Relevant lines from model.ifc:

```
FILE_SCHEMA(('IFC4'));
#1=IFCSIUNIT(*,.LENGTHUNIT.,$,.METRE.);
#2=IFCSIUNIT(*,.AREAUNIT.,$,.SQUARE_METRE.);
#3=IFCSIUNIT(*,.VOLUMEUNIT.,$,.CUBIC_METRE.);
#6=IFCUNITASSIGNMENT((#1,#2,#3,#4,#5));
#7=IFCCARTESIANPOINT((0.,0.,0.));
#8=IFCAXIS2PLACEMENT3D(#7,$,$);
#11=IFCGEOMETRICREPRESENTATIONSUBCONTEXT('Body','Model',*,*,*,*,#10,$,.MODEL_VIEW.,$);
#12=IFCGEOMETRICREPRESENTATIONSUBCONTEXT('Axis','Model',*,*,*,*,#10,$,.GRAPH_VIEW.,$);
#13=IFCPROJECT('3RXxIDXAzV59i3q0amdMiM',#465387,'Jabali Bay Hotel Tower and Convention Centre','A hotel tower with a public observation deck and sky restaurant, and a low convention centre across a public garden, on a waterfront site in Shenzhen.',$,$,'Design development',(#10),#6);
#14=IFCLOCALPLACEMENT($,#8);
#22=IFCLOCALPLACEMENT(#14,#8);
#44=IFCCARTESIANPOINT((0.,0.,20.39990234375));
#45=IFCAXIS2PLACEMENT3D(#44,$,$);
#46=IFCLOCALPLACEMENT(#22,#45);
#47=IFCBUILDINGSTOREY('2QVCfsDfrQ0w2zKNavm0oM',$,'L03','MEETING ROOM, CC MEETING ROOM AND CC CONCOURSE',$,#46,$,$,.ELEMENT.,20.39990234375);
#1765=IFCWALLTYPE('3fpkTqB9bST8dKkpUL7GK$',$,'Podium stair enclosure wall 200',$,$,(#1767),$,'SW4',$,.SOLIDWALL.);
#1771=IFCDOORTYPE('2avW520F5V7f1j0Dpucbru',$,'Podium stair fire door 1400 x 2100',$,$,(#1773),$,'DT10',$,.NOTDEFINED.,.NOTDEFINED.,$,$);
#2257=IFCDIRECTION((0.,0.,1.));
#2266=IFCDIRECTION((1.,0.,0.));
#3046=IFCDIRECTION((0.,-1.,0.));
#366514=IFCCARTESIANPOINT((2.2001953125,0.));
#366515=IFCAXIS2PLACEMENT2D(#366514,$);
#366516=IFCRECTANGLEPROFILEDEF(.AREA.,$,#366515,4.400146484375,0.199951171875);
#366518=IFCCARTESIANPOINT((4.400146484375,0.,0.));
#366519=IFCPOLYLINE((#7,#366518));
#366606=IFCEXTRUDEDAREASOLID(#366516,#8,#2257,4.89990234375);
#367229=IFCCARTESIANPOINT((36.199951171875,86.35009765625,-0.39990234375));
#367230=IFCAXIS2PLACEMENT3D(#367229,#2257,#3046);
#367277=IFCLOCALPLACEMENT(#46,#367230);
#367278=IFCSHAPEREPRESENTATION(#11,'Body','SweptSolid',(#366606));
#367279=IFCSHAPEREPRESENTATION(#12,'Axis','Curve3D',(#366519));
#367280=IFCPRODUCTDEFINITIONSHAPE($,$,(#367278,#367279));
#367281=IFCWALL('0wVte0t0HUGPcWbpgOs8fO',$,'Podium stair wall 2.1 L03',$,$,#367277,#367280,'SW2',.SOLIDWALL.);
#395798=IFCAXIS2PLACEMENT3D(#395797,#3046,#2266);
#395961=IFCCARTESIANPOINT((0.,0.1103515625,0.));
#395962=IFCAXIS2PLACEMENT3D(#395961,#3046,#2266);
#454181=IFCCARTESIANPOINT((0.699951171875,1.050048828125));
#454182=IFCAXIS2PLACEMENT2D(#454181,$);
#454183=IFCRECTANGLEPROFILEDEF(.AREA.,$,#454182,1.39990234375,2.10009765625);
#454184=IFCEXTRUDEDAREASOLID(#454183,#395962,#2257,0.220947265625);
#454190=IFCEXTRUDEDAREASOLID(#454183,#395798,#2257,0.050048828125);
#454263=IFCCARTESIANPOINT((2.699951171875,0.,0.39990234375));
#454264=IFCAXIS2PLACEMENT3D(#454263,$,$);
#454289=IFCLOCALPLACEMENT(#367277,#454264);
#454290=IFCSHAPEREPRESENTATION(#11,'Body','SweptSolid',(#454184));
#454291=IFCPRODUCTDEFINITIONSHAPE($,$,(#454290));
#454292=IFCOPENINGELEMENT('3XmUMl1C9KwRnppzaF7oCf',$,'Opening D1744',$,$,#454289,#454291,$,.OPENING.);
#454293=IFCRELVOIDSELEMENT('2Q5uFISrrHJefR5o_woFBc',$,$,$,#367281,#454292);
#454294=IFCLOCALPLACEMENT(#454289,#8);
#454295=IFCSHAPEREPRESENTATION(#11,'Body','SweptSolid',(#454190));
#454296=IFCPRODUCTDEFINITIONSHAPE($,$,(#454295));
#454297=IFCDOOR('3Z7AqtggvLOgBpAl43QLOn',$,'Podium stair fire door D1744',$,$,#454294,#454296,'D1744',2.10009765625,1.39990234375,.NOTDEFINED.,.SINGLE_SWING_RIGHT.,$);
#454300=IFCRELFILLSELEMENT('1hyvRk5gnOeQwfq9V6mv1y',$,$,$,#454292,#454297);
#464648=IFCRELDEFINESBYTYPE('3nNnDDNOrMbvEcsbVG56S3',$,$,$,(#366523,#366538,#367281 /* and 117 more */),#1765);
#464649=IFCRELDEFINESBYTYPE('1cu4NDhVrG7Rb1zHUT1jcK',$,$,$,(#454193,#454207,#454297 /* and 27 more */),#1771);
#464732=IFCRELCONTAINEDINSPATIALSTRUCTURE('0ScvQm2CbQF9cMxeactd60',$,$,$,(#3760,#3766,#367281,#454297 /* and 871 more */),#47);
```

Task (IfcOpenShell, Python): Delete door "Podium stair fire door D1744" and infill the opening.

```python
import ifcopenshell
import ifcopenshell.api.feature
import ifcopenshell.api.root
import ifcopenshell.geom
import ifcopenshell.util.shape

model = ifcopenshell.open("model.ifc")
settings = ifcopenshell.geom.settings()


def volume(element):
    """Net volume in cubic metres, openings subtracted."""
    shape = ifcopenshell.geom.create_shape(settings, element)
    return ifcopenshell.util.shape.get_volume(shape.geometry)


door = model.by_guid("3Z7AqtggvLOgBpAl43QLOn")
opening = door.FillsVoids[0].RelatingOpeningElement
wall = opening.VoidsElements[0].RelatingBuildingElement
before = volume(wall)

ifcopenshell.api.root.remove_product(model, product=door)
ifcopenshell.api.feature.remove_feature(model, feature=opening)

after = volume(wall)

print(f"wall volume {before:.3f} -> {after:.3f} m3")

model.write("model_updated.ifc")
```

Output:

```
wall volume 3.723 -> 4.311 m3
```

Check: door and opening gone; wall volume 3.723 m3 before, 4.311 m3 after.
